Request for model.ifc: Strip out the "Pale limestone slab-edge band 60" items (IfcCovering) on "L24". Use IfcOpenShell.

First a look at what the model holds.

```python
import ifcopenshell
import ifcopenshell.util.element

model = ifcopenshell.open("model.ifc")
print(model.schema)
storey = next(s for s in model.by_type("IfcBuildingStorey") if s.Name == "L24")
coverings = [e for e in ifcopenshell.util.element.get_decomposition(storey) if e.is_a("IfcCovering")]
seen = {}
for e in coverings:
    element_type = ifcopenshell.util.element.get_type(e)
    name = element_type.Name if element_type not in (None, e) else None
    seen[name] = seen.get(name, 0) + 1
for name, count in sorted(seen.items(), key=str):
    print(count, "x", name)
```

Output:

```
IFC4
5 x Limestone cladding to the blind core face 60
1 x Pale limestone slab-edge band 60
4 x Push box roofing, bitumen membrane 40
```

```python
import ifcopenshell
import ifcopenshell.api.root
import ifcopenshell.util.element

model = ifcopenshell.open("model.ifc")

storey = next(s for s in model.by_type("IfcBuildingStorey") if s.Name == "L24")
coverings = [e for e in ifcopenshell.util.element.get_decomposition(storey) if e.is_a("IfcCovering")]
targets = [e for e in coverings if (t := ifcopenshell.util.element.get_type(e)) not in (None, e) and t.Name == "Pale limestone slab-edge band 60"]

for e in targets:
    ifcopenshell.api.root.remove_product(model, product=e)
print(len(targets), "removed")

model.write("model-out.ifc")
```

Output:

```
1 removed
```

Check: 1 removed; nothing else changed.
